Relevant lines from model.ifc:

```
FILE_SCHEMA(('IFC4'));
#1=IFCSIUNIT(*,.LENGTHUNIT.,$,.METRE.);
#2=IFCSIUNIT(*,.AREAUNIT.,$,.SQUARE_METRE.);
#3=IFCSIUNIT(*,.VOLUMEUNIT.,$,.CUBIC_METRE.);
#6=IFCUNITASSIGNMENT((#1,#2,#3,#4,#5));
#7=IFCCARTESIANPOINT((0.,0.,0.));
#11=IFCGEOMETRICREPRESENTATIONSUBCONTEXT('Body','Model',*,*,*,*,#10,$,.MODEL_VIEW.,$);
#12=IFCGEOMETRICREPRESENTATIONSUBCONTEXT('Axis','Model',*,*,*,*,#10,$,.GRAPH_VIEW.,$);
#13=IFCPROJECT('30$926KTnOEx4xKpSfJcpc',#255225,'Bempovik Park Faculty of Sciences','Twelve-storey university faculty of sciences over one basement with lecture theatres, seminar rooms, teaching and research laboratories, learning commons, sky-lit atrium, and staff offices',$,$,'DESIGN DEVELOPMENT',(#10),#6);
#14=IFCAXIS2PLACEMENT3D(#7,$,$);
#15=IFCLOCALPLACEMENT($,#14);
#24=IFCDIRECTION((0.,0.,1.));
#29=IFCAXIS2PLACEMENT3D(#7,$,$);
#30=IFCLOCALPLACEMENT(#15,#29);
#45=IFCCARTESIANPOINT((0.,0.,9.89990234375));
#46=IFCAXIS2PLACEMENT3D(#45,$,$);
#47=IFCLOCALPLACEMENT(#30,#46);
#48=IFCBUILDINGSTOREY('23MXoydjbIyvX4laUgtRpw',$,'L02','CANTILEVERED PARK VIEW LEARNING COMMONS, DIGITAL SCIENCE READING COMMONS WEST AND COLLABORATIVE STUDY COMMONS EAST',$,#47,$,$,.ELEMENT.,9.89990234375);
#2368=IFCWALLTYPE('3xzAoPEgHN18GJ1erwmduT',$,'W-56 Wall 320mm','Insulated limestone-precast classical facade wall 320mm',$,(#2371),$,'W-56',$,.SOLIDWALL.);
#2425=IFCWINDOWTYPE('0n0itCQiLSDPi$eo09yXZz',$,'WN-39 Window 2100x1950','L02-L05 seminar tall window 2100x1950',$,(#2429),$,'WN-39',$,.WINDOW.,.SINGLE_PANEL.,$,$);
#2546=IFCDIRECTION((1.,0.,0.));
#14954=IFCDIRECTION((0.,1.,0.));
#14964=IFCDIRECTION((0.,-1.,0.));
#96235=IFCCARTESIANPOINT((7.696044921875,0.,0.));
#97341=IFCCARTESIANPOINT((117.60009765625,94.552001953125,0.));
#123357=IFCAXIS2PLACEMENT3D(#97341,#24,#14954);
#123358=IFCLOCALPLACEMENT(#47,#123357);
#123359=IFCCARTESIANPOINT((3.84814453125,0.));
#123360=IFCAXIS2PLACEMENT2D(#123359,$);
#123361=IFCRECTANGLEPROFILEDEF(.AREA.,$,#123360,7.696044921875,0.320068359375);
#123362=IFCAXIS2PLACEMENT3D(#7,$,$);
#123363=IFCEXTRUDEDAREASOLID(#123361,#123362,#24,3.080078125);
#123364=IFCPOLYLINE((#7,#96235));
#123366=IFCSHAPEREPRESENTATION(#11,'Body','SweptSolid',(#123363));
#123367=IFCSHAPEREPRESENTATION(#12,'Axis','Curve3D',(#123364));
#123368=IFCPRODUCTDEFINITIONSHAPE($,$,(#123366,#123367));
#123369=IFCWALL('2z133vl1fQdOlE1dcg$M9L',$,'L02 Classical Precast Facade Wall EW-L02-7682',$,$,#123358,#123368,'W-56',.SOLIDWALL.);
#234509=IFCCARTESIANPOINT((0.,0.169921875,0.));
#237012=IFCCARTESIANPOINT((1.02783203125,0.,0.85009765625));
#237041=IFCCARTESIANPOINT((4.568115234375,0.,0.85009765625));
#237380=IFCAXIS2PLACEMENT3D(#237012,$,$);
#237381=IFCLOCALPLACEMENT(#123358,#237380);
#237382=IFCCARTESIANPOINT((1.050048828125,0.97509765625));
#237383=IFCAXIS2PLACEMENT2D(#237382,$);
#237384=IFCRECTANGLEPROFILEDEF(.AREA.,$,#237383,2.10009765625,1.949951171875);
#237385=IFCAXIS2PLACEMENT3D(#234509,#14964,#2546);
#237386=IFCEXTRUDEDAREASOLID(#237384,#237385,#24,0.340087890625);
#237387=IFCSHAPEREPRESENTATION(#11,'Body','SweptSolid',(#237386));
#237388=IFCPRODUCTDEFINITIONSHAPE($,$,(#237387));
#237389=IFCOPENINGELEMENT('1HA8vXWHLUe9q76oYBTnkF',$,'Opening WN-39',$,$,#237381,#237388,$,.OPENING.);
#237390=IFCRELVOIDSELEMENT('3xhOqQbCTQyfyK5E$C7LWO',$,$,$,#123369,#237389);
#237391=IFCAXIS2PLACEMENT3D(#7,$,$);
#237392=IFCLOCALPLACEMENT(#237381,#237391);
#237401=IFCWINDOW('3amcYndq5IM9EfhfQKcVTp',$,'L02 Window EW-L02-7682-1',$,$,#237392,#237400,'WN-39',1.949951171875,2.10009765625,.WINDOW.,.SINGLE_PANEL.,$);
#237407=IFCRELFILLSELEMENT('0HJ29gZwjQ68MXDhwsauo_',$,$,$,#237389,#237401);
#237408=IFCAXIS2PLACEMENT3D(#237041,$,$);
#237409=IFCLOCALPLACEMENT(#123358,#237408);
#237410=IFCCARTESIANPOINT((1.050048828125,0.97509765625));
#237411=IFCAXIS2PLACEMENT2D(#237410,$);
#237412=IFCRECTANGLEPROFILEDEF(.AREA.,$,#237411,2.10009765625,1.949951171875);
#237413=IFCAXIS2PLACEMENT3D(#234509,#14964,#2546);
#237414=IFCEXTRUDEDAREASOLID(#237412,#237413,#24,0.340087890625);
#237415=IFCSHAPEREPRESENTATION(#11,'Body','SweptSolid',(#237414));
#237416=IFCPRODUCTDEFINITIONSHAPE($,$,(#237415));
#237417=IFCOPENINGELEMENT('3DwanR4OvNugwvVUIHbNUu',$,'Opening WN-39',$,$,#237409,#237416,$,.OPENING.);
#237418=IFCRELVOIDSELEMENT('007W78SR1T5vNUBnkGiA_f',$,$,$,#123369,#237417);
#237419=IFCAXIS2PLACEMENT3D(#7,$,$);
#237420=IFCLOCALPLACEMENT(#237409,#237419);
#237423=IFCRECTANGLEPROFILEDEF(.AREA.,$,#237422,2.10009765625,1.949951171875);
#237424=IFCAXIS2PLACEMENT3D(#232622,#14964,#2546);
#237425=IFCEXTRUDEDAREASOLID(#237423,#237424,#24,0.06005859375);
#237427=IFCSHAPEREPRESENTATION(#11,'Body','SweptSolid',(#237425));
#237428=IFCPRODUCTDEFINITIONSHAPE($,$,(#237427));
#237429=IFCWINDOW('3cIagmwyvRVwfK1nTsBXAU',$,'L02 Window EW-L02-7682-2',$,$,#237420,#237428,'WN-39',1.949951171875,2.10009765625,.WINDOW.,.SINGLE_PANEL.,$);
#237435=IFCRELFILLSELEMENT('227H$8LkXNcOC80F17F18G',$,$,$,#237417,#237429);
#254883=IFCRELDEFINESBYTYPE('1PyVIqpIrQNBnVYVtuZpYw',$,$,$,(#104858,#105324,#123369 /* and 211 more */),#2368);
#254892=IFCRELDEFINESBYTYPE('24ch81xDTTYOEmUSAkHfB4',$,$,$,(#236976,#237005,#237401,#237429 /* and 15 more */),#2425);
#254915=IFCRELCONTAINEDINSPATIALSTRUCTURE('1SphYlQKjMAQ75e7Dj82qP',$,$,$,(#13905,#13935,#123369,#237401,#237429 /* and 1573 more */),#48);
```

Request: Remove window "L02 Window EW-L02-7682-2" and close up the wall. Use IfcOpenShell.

```python
import ifcopenshell
import ifcopenshell.api.feature
import ifcopenshell.api.root
import ifcopenshell.geom
import ifcopenshell.util.shape

model = ifcopenshell.open("model.ifc")
settings = ifcopenshell.geom.settings()


def volume(element):
    """Net volume in cubic metres, openings subtracted."""
    shape = ifcopenshell.geom.create_shape(settings, element)
    return ifcopenshell.util.shape.get_volume(shape.geometry)


window = model.by_guid("3cIagmwyvRVwfK1nTsBXAU")
opening = window.FillsVoids[0].RelatingOpeningElement
wall = opening.VoidsElements[0].RelatingBuildingElement
before = volume(wall)

ifcopenshell.api.root.remove_product(model, product=window)
ifcopenshell.api.feature.remove_feature(model, feature=opening)

after = volume(wall)

print(f"wall volume {before:.3f} -> {after:.3f} m3")

model.write("model_updated.ifc")
```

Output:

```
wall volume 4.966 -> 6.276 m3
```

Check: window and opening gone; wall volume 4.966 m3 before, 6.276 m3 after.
